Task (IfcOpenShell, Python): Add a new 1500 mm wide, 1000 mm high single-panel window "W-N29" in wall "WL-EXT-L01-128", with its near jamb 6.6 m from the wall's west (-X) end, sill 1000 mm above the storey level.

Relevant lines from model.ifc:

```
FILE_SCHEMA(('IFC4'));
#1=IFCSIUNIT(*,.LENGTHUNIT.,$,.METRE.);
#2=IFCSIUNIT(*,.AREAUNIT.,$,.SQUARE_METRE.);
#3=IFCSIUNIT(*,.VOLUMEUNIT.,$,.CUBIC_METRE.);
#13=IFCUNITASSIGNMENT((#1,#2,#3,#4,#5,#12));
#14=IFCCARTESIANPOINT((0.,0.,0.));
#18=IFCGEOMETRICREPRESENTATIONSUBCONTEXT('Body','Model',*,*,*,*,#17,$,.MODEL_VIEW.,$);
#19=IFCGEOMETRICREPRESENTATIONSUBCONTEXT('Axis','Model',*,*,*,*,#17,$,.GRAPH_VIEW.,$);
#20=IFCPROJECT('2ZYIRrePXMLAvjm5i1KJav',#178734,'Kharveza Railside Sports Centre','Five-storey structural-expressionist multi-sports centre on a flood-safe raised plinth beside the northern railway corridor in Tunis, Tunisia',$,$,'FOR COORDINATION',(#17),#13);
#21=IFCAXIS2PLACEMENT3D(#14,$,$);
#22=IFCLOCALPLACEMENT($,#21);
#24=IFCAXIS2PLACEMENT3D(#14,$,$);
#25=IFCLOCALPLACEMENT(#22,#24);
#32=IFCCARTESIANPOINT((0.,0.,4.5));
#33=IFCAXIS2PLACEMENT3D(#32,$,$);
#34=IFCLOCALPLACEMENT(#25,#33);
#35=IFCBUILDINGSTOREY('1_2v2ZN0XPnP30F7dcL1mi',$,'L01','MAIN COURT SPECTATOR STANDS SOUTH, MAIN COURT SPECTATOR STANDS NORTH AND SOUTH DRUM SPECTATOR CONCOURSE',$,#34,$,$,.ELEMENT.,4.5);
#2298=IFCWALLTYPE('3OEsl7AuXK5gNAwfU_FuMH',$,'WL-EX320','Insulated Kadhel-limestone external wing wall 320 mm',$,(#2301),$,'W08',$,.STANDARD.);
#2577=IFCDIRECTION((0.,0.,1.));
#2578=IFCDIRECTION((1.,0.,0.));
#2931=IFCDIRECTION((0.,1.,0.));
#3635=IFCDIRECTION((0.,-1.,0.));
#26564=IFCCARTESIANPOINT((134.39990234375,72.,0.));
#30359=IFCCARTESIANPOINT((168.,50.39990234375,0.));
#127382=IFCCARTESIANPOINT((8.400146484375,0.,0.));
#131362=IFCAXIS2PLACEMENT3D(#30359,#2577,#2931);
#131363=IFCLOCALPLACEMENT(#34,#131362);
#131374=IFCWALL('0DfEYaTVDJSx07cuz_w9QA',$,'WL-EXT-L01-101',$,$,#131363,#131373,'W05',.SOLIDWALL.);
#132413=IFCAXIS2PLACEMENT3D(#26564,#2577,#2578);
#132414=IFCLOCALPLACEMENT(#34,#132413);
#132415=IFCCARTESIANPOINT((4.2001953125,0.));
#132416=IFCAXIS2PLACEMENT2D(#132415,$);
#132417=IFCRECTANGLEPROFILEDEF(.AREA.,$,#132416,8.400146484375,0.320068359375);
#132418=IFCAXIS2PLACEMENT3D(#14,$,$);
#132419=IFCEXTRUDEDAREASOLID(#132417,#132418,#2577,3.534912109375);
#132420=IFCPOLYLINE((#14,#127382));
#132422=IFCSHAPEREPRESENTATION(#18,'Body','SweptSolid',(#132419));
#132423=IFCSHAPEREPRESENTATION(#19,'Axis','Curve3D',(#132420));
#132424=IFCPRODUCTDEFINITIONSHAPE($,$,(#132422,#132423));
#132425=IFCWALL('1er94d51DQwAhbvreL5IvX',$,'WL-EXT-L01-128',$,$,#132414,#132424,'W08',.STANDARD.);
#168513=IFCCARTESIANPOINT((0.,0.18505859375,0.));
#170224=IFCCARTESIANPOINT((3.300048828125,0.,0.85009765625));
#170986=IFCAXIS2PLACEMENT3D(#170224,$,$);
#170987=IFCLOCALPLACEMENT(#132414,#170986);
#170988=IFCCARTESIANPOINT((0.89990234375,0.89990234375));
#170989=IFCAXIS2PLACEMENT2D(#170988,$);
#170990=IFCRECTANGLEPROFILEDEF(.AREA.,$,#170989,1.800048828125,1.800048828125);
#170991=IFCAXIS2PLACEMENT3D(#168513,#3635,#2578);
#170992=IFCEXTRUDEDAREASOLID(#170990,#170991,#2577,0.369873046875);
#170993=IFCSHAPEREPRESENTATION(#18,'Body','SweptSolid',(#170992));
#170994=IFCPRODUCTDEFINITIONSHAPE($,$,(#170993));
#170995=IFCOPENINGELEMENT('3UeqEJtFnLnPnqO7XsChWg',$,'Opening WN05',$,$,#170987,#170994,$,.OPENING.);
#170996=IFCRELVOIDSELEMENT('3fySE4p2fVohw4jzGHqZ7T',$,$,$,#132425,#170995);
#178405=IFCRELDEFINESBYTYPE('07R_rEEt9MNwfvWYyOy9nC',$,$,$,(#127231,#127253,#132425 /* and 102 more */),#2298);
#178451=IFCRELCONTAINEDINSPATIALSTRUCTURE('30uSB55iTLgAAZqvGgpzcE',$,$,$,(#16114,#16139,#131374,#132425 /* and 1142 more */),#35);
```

```python
import numpy as np
import ifcopenshell
import ifcopenshell.api.feature
import ifcopenshell.api.geometry
import ifcopenshell.api.root
import ifcopenshell.api.spatial
import ifcopenshell.geom
import ifcopenshell.util.element
import ifcopenshell.util.placement
import ifcopenshell.util.representation
import ifcopenshell.util.shape
import ifcopenshell.util.unit

model = ifcopenshell.open("model.ifc")
unit_scale = ifcopenshell.util.unit.calculate_unit_scale(model)
settings = ifcopenshell.geom.settings()


def volume(element):
    """Net volume in cubic metres, openings subtracted."""
    shape = ifcopenshell.geom.create_shape(settings, element)
    return ifcopenshell.util.shape.get_volume(shape.geometry)


wall = model.by_guid("1er94d51DQwAhbvreL5IvX")
storey = ifcopenshell.util.element.get_container(wall, ifc_class="IfcBuildingStorey")
context = ifcopenshell.util.representation.get_context(model, "Model", "Body", "MODEL_VIEW")
before = volume(wall)

width, height, from_end, sill = 1.5, 1, 6.6, 1  # metres

# The wall runs along its own X axis, and the end named is its -X end.
wall_shape = ifcopenshell.geom.create_shape(settings, wall)
x, y, z = ifcopenshell.util.shape.get_vertices(wall_shape.geometry).T
start = x.min() + from_end
face, thickness = float(y.min()), float(y.max() - y.min())
wall_matrix = ifcopenshell.util.placement.get_local_placement(wall.ObjectPlacement)
level = ifcopenshell.util.placement.get_local_placement(storey.ObjectPlacement)[2, 3]


def in_wall(x, y):
    """Placement at x, y metres in the wall's axes, at sill height."""
    matrix = wall_matrix.copy()
    matrix[:, 3] = wall_matrix @ np.array([x / unit_scale, y / unit_scale, 0.0, 1.0])
    matrix[2, 3] = level + sill / unit_scale
    return matrix


# Opening: a box that overshoots both wall faces by 50 mm.
opening = ifcopenshell.api.root.create_entity(model, ifc_class="IfcOpeningElement", predefined_type="OPENING")
box = ifcopenshell.api.geometry.add_wall_representation(
    model, context=context, length=width, height=height, thickness=thickness + 0.1
)
ifcopenshell.api.geometry.assign_representation(model, product=opening, representation=box)
ifcopenshell.api.geometry.edit_object_placement(model, product=opening, matrix=in_wall(start, face - 0.05), is_si=False)
ifcopenshell.api.feature.add_feature(model, feature=opening, element=wall)

window = ifcopenshell.api.root.create_entity(model, ifc_class="IfcWindow", name="W-N29", predefined_type="WINDOW")
window.OverallWidth, window.OverallHeight = width / unit_scale, height / unit_scale
window.PartitioningType = "SINGLE_PANEL"
body = ifcopenshell.api.geometry.add_window_representation(
    model,
    context=context,
    overall_width=window.OverallWidth,
    overall_height=window.OverallHeight,
    partition_type="SINGLE_PANEL",
)
ifcopenshell.api.geometry.assign_representation(model, product=window, representation=body)
ifcopenshell.api.spatial.assign_container(model, products=[window], relating_structure=storey)
ifcopenshell.api.feature.add_filling(model, opening=opening, element=window)

# Centre the window in the wall's thickness.
ifcopenshell.api.geometry.edit_object_placement(model, product=window, matrix=in_wall(start, face), is_si=False)
window_shape = ifcopenshell.geom.create_shape(settings, window)
depth = ifcopenshell.util.shape.get_vertices(window_shape.geometry)[:, 1]
offset = face + thickness / 2 - (depth.min() + depth.max()) / 2
ifcopenshell.api.geometry.edit_object_placement(model, product=window, matrix=in_wall(start, offset), is_si=False)

after = volume(wall)

print(f"wall volume {before:.3f} -> {after:.3f} m3")

model.write("model_edited.ifc")
```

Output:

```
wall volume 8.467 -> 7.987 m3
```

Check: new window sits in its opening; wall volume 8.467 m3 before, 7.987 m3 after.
